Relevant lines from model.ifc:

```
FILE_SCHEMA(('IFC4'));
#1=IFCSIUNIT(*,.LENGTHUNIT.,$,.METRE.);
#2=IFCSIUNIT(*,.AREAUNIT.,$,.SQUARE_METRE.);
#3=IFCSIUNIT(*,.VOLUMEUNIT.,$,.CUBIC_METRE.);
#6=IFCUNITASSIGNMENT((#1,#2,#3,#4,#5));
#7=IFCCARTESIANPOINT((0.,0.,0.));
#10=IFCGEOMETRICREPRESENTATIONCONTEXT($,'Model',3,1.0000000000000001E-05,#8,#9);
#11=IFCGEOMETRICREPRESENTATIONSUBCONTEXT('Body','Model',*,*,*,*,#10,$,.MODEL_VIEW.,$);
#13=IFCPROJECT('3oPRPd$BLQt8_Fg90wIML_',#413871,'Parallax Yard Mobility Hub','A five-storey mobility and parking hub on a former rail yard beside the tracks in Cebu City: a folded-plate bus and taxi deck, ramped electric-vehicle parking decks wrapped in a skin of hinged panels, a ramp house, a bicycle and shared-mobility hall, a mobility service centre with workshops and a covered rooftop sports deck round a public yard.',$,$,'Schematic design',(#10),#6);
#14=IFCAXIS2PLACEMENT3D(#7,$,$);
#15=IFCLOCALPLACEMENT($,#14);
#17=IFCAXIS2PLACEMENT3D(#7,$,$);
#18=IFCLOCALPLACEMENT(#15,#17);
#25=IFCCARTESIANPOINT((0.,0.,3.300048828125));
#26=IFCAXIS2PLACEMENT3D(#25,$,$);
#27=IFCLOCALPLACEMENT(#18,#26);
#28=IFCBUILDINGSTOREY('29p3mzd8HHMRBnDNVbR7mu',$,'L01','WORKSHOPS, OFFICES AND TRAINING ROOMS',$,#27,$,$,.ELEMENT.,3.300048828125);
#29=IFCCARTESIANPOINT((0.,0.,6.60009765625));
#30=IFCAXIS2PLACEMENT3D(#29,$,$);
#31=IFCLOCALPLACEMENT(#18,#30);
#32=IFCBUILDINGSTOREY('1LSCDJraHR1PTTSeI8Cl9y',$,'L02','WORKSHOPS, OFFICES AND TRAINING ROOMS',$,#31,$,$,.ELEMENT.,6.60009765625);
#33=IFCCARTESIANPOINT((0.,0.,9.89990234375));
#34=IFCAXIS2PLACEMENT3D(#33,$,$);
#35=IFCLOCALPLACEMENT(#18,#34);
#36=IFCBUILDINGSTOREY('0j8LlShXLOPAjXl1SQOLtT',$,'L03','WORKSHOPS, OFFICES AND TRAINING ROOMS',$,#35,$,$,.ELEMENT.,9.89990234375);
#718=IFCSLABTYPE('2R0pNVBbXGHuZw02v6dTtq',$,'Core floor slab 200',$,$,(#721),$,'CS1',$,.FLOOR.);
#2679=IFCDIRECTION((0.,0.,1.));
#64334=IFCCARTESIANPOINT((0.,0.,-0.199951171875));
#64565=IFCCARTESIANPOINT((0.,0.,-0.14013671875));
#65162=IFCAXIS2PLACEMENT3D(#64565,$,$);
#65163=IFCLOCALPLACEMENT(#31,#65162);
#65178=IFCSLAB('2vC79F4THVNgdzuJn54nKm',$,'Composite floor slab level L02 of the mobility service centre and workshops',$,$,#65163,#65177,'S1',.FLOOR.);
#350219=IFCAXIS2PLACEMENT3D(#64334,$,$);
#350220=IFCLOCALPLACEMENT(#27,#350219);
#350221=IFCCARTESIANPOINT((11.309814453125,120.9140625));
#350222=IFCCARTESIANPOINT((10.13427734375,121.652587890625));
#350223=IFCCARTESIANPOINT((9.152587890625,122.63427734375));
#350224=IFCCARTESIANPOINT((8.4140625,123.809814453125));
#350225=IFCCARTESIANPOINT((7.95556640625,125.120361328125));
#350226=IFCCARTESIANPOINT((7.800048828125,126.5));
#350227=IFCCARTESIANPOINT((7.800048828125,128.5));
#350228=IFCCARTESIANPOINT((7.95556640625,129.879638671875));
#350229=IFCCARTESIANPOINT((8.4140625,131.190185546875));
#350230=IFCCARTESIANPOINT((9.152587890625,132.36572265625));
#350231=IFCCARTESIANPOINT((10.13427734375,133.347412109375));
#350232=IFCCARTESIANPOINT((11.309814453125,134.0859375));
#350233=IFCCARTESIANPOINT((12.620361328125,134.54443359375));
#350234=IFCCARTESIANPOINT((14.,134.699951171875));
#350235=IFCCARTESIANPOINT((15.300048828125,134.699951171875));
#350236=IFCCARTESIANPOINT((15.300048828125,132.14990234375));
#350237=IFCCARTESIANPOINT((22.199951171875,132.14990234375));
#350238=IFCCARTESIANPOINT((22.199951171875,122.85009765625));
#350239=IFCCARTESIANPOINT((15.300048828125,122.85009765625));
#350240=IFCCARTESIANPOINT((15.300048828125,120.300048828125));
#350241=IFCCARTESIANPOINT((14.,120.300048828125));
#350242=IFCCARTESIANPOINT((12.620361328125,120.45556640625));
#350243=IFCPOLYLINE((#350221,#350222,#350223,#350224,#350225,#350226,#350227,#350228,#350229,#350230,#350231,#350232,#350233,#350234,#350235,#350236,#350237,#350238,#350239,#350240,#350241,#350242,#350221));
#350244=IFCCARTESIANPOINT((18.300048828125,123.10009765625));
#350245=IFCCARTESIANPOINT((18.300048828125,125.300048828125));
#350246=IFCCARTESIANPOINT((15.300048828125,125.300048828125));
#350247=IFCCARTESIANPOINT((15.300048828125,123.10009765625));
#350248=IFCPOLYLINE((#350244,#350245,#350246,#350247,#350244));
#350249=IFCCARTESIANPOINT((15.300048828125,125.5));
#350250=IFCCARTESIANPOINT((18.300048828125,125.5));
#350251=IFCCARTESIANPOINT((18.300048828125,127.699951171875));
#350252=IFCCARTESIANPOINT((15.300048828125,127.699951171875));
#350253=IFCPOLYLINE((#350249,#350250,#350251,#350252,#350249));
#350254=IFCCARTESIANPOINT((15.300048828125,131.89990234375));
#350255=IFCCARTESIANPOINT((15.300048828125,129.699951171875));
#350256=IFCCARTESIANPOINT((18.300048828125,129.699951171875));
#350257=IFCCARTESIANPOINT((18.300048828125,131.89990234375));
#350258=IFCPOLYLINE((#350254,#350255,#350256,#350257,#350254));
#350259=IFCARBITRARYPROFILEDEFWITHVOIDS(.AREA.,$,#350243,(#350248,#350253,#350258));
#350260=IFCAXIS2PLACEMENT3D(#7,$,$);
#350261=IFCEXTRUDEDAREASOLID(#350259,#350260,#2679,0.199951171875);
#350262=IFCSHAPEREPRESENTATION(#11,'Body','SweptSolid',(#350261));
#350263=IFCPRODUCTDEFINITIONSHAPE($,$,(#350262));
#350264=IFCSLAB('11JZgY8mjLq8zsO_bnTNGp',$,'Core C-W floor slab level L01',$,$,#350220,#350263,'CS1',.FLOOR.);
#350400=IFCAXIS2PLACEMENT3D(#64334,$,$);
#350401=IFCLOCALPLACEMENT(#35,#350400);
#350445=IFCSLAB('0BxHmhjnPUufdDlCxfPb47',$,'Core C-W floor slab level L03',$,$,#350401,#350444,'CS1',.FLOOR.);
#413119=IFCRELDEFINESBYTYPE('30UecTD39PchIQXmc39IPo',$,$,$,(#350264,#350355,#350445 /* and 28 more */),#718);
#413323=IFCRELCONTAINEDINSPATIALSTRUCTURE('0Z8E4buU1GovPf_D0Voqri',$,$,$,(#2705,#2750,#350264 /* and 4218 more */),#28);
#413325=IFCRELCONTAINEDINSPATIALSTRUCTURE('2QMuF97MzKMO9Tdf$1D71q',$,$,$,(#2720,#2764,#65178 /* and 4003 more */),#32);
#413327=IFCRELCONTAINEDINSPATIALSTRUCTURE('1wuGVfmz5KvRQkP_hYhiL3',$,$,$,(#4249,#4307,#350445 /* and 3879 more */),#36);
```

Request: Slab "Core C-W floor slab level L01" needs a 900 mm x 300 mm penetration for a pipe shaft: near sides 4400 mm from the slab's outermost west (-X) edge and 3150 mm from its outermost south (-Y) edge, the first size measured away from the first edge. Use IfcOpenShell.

```python
import numpy as np
import ifcopenshell
import ifcopenshell.api.feature
import ifcopenshell.api.geometry
import ifcopenshell.api.root
import ifcopenshell.geom
import ifcopenshell.util.placement
import ifcopenshell.util.representation
import ifcopenshell.util.shape
import ifcopenshell.util.unit

model = ifcopenshell.open("model.ifc")
unit_scale = ifcopenshell.util.unit.calculate_unit_scale(model)
settings = ifcopenshell.geom.settings()


def volume(element):
    """Net volume in cubic metres, openings subtracted."""
    shape = ifcopenshell.geom.create_shape(settings, element)
    return ifcopenshell.util.shape.get_volume(shape.geometry)


slab = model.by_id(350264)
before = volume(slab)

# Extent in the slab's own axes, in metres. The edges named are its -X and -Y sides.
slab_shape = ifcopenshell.geom.create_shape(settings, slab)
vertices = ifcopenshell.util.shape.get_vertices(slab_shape.geometry)
x_min, y_min, bottom = vertices.min(axis=0)
top = vertices[:, 2].max()

opening = ifcopenshell.api.root.create_entity(model, ifc_class="IfcOpeningElement", name="Pipe shaft opening", predefined_type="OPENING")
context = ifcopenshell.util.representation.get_context(model, "Model", "Body", "MODEL_VIEW")
width, depth = 0.9, 0.3
outline = [(0.0, 0.0), (width, 0.0), (width, depth), (0.0, depth), (0.0, 0.0)]
# Overshoot both faces by 50 mm so the cut is clean.
shape = ifcopenshell.api.geometry.add_slab_representation(
    model, context=context, depth=top - bottom + 0.1, polyline=outline
)
ifcopenshell.api.geometry.assign_representation(model, product=opening, representation=shape)

matrix = ifcopenshell.util.placement.get_local_placement(slab.ObjectPlacement)
matrix[:, 3] = matrix @ np.append(np.array([x_min + 4.4, y_min + 3.15, bottom - 0.05]) / unit_scale, 1.0)
ifcopenshell.api.geometry.edit_object_placement(model, product=opening, matrix=matrix, is_si=False)
ifcopenshell.api.feature.add_feature(model, feature=opening, element=slab)

after = volume(slab)

print(f"slab volume {before:.3f} -> {after:.3f} m3")

model.write("model-out.ifc")
```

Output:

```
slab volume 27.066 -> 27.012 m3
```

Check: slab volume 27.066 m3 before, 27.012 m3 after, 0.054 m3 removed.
